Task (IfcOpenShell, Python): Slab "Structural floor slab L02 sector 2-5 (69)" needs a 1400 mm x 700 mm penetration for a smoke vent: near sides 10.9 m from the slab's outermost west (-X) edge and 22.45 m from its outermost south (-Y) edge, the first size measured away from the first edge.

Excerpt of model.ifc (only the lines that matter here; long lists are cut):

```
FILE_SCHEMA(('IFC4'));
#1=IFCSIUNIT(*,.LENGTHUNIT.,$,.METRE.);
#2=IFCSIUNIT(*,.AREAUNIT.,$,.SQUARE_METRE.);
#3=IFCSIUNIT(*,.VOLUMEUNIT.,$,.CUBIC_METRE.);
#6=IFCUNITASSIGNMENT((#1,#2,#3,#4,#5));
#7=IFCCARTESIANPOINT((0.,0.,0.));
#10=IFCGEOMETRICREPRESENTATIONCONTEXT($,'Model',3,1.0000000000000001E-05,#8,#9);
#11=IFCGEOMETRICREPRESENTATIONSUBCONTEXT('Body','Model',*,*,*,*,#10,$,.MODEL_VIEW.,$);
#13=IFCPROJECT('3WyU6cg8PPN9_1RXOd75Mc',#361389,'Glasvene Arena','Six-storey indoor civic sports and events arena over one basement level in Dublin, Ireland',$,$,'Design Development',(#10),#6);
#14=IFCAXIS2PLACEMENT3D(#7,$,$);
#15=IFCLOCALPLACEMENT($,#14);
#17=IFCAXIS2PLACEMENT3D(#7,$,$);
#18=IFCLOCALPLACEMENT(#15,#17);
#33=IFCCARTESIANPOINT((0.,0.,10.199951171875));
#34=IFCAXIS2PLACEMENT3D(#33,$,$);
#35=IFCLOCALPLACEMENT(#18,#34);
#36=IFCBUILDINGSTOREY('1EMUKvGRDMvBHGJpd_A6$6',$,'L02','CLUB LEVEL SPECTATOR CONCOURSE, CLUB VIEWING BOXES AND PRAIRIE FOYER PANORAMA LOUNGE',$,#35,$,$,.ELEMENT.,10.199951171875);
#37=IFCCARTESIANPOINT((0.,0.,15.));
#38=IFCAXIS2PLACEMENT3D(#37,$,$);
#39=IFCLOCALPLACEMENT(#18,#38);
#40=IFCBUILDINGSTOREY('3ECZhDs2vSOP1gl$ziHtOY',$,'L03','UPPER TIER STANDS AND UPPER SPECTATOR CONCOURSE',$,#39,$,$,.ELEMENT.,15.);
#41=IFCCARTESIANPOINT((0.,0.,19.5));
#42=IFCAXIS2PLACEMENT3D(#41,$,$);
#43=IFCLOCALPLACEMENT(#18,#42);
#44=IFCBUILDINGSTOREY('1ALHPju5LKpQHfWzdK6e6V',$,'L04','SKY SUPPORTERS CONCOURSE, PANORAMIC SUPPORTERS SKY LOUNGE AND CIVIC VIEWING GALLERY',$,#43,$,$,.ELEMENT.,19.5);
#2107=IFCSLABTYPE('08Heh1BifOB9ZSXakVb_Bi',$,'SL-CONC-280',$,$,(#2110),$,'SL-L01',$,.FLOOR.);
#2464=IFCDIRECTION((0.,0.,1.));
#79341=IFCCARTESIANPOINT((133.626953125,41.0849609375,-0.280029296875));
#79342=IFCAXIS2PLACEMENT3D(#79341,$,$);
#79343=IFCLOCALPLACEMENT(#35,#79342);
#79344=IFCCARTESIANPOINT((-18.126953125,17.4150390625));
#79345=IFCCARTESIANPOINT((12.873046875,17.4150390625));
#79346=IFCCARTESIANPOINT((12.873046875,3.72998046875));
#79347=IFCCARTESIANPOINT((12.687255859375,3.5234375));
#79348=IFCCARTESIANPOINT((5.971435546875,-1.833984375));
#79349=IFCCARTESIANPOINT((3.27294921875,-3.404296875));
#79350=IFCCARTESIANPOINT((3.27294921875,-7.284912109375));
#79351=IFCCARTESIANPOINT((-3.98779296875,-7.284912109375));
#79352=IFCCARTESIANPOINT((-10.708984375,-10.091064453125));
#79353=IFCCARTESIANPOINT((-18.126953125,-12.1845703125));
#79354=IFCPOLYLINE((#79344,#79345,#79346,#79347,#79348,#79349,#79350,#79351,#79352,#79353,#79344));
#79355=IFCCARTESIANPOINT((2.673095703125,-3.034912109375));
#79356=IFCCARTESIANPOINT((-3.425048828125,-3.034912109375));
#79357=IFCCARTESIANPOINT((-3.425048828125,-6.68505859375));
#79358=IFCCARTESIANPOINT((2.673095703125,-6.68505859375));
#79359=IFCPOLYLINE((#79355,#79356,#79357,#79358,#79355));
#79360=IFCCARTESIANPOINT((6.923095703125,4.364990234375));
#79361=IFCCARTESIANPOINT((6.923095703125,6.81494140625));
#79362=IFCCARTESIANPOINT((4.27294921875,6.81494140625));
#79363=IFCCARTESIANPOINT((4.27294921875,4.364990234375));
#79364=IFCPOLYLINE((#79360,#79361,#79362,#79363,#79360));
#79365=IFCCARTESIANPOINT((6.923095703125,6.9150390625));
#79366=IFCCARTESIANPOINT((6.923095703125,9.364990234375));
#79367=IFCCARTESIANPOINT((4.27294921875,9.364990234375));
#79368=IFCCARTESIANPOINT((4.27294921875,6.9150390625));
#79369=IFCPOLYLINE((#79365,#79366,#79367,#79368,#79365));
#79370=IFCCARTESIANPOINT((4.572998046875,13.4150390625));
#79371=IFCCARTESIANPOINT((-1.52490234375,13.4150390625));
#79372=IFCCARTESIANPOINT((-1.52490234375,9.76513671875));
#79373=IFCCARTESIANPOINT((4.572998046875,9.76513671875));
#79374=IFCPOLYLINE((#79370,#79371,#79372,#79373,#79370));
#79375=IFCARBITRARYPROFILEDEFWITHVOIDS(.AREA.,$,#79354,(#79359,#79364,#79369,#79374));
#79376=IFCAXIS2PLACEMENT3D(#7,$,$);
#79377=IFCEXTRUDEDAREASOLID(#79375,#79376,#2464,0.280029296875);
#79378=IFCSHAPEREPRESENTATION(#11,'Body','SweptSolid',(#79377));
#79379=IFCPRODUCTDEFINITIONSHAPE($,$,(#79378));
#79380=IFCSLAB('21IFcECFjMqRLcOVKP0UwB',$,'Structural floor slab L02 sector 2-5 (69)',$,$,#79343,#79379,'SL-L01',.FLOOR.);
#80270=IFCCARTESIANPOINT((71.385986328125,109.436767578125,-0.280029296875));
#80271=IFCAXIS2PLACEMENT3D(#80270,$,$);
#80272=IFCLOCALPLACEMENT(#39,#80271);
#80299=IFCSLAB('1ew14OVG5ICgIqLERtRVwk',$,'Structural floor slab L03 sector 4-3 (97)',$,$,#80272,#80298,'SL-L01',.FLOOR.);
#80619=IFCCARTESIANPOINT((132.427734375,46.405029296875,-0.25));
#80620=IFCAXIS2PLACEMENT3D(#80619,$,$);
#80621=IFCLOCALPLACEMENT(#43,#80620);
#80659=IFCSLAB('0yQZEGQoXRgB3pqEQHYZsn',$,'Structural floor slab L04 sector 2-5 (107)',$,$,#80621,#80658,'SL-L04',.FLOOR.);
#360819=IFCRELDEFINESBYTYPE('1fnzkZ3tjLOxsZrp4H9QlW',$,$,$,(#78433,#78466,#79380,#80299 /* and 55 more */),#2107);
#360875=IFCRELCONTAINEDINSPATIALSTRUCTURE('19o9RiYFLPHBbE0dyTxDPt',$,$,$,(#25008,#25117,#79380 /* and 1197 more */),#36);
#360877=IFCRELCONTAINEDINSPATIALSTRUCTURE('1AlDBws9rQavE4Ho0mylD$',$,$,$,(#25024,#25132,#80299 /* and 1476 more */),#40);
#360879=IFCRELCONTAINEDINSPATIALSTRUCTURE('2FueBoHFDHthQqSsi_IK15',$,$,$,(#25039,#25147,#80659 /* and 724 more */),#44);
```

```python
import numpy as np
import ifcopenshell
import ifcopenshell.api.feature
import ifcopenshell.api.geometry
import ifcopenshell.api.root
import ifcopenshell.geom
import ifcopenshell.util.placement
import ifcopenshell.util.representation
import ifcopenshell.util.shape
import ifcopenshell.util.unit

model = ifcopenshell.open("model.ifc")
unit_scale = ifcopenshell.util.unit.calculate_unit_scale(model)
settings = ifcopenshell.geom.settings()


def volume(element):
    """Net volume in cubic metres, openings subtracted."""
    shape = ifcopenshell.geom.create_shape(settings, element)
    return ifcopenshell.util.shape.get_volume(shape.geometry)


slab = model.by_guid("21IFcECFjMqRLcOVKP0UwB")
before = volume(slab)

# Extent in the slab's own axes, in metres. The edges named are its -X and -Y sides.
slab_shape = ifcopenshell.geom.create_shape(settings, slab)
vertices = ifcopenshell.util.shape.get_vertices(slab_shape.geometry)
x_min, y_min, bottom = vertices.min(axis=0)
top = vertices[:, 2].max()

opening = ifcopenshell.api.root.create_entity(model, ifc_class="IfcOpeningElement", name="Smoke vent opening", predefined_type="OPENING")
context = ifcopenshell.util.representation.get_context(model, "Model", "Body", "MODEL_VIEW")
width, depth = 1.4, 0.7
outline = [(0.0, 0.0), (width, 0.0), (width, depth), (0.0, depth), (0.0, 0.0)]
# Overshoot both faces by 50 mm so the cut is clean.
shape = ifcopenshell.api.geometry.add_slab_representation(
    model, context=context, depth=top - bottom + 0.1, polyline=outline
)
ifcopenshell.api.geometry.assign_representation(model, product=opening, representation=shape)

matrix = ifcopenshell.util.placement.get_local_placement(slab.ObjectPlacement)
matrix[:, 3] = matrix @ np.append(np.array([x_min + 10.9, y_min + 22.45, bottom - 0.05]) / unit_scale, 1.0)
ifcopenshell.api.geometry.edit_object_placement(model, product=opening, matrix=matrix, is_si=False)
ifcopenshell.api.feature.add_feature(model, feature=opening, element=slab)

after = volume(slab)

print(f"slab volume {before:.3f} -> {after:.3f} m3")

model.write("model_updated.ifc")
```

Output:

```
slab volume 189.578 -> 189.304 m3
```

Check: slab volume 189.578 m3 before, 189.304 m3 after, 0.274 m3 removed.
